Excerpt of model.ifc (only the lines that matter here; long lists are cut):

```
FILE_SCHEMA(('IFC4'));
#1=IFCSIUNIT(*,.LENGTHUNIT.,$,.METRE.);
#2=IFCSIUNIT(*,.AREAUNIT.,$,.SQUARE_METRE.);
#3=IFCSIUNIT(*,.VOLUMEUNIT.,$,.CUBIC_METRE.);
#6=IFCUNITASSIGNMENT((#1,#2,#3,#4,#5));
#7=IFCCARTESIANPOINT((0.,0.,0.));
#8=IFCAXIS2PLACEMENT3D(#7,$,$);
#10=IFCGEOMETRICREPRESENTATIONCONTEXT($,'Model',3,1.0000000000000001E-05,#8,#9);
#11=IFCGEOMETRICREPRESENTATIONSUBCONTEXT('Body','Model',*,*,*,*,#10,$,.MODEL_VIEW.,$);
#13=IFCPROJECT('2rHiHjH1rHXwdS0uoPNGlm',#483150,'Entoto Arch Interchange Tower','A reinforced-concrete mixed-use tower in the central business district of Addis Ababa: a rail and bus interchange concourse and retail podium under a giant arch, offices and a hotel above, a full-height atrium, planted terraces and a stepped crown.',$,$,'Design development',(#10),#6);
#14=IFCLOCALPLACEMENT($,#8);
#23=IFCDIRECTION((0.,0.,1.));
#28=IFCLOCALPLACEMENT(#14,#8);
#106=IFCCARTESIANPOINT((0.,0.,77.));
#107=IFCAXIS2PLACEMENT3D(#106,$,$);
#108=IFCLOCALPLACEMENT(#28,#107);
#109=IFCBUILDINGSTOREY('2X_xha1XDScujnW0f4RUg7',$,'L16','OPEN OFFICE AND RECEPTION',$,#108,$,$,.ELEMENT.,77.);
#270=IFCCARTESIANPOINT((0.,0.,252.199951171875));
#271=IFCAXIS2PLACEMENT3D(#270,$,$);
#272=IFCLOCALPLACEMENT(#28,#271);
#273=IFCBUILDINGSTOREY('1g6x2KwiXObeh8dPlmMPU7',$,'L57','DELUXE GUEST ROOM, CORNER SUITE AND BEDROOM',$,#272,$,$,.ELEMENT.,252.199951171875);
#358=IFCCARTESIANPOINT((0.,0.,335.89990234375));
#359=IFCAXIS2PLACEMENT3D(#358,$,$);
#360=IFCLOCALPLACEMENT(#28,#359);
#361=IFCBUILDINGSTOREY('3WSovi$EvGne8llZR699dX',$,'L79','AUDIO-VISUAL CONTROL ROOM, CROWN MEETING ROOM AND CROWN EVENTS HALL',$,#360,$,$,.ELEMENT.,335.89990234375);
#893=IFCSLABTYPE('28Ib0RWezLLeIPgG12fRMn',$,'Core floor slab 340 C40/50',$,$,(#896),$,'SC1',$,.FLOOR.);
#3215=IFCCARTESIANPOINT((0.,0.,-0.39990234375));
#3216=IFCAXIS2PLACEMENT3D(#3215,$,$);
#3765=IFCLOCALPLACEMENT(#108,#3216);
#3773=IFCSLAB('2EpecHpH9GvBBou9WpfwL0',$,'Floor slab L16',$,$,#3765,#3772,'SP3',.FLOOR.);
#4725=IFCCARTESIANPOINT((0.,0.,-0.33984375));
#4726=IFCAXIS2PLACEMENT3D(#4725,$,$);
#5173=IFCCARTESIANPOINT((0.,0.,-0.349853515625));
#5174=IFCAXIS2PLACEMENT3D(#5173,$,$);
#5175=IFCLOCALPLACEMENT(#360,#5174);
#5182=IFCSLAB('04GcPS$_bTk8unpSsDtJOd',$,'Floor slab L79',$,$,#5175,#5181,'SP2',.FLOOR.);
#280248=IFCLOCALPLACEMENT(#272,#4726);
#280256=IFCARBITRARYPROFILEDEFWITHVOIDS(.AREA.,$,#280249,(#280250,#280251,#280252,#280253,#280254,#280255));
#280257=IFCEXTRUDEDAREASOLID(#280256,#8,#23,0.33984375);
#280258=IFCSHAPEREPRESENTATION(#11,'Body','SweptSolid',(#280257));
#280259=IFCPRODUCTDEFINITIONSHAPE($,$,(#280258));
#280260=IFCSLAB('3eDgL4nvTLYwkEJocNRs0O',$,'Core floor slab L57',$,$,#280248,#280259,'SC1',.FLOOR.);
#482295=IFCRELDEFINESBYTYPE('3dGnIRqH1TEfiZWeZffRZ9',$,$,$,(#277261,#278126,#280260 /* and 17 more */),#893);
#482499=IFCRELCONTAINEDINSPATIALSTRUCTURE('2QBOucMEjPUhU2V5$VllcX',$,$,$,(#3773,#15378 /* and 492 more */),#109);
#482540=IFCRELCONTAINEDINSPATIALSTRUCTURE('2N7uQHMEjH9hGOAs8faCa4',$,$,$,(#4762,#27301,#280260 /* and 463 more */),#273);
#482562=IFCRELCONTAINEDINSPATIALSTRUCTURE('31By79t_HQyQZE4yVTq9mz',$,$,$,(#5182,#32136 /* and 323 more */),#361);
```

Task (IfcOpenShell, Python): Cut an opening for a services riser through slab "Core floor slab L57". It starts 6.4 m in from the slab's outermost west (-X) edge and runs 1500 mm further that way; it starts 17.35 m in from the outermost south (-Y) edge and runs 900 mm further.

```python
import numpy as np
import ifcopenshell
import ifcopenshell.api.feature
import ifcopenshell.api.geometry
import ifcopenshell.api.root
import ifcopenshell.geom
import ifcopenshell.util.placement
import ifcopenshell.util.representation
import ifcopenshell.util.shape
import ifcopenshell.util.unit

model = ifcopenshell.open("model.ifc")
unit_scale = ifcopenshell.util.unit.calculate_unit_scale(model)
settings = ifcopenshell.geom.settings()


def volume(element):
    """Net volume in cubic metres, openings subtracted."""
    shape = ifcopenshell.geom.create_shape(settings, element)
    return ifcopenshell.util.shape.get_volume(shape.geometry)


slab = model.by_guid("3eDgL4nvTLYwkEJocNRs0O")
before = volume(slab)

# Extent in the slab's own axes, in metres. The edges named are its -X and -Y sides.
slab_shape = ifcopenshell.geom.create_shape(settings, slab)
vertices = ifcopenshell.util.shape.get_vertices(slab_shape.geometry)
x_min, y_min, bottom = vertices.min(axis=0)
top = vertices[:, 2].max()

opening = ifcopenshell.api.root.create_entity(model, ifc_class="IfcOpeningElement", name="Services riser opening", predefined_type="OPENING")
context = ifcopenshell.util.representation.get_context(model, "Model", "Body", "MODEL_VIEW")
width, depth = 1.5, 0.9
outline = [(0.0, 0.0), (width, 0.0), (width, depth), (0.0, depth), (0.0, 0.0)]
# Overshoot both faces by 50 mm so the cut is clean.
shape = ifcopenshell.api.geometry.add_slab_representation(
    model, context=context, depth=top - bottom + 0.1, polyline=outline
)
ifcopenshell.api.geometry.assign_representation(model, product=opening, representation=shape)

matrix = ifcopenshell.util.placement.get_local_placement(slab.ObjectPlacement)
matrix[:, 3] = matrix @ np.append(np.array([x_min + 6.4, y_min + 17.35, bottom - 0.05]) / unit_scale, 1.0)
ifcopenshell.api.geometry.edit_object_placement(model, product=opening, matrix=matrix, is_si=False)
ifcopenshell.api.feature.add_feature(model, feature=opening, element=slab)

after = volume(slab)

print(f"slab volume {before:.3f} -> {after:.3f} m3")

model.write("model-out.ifc")
```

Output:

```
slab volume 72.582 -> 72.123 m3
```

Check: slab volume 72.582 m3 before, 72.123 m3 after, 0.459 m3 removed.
